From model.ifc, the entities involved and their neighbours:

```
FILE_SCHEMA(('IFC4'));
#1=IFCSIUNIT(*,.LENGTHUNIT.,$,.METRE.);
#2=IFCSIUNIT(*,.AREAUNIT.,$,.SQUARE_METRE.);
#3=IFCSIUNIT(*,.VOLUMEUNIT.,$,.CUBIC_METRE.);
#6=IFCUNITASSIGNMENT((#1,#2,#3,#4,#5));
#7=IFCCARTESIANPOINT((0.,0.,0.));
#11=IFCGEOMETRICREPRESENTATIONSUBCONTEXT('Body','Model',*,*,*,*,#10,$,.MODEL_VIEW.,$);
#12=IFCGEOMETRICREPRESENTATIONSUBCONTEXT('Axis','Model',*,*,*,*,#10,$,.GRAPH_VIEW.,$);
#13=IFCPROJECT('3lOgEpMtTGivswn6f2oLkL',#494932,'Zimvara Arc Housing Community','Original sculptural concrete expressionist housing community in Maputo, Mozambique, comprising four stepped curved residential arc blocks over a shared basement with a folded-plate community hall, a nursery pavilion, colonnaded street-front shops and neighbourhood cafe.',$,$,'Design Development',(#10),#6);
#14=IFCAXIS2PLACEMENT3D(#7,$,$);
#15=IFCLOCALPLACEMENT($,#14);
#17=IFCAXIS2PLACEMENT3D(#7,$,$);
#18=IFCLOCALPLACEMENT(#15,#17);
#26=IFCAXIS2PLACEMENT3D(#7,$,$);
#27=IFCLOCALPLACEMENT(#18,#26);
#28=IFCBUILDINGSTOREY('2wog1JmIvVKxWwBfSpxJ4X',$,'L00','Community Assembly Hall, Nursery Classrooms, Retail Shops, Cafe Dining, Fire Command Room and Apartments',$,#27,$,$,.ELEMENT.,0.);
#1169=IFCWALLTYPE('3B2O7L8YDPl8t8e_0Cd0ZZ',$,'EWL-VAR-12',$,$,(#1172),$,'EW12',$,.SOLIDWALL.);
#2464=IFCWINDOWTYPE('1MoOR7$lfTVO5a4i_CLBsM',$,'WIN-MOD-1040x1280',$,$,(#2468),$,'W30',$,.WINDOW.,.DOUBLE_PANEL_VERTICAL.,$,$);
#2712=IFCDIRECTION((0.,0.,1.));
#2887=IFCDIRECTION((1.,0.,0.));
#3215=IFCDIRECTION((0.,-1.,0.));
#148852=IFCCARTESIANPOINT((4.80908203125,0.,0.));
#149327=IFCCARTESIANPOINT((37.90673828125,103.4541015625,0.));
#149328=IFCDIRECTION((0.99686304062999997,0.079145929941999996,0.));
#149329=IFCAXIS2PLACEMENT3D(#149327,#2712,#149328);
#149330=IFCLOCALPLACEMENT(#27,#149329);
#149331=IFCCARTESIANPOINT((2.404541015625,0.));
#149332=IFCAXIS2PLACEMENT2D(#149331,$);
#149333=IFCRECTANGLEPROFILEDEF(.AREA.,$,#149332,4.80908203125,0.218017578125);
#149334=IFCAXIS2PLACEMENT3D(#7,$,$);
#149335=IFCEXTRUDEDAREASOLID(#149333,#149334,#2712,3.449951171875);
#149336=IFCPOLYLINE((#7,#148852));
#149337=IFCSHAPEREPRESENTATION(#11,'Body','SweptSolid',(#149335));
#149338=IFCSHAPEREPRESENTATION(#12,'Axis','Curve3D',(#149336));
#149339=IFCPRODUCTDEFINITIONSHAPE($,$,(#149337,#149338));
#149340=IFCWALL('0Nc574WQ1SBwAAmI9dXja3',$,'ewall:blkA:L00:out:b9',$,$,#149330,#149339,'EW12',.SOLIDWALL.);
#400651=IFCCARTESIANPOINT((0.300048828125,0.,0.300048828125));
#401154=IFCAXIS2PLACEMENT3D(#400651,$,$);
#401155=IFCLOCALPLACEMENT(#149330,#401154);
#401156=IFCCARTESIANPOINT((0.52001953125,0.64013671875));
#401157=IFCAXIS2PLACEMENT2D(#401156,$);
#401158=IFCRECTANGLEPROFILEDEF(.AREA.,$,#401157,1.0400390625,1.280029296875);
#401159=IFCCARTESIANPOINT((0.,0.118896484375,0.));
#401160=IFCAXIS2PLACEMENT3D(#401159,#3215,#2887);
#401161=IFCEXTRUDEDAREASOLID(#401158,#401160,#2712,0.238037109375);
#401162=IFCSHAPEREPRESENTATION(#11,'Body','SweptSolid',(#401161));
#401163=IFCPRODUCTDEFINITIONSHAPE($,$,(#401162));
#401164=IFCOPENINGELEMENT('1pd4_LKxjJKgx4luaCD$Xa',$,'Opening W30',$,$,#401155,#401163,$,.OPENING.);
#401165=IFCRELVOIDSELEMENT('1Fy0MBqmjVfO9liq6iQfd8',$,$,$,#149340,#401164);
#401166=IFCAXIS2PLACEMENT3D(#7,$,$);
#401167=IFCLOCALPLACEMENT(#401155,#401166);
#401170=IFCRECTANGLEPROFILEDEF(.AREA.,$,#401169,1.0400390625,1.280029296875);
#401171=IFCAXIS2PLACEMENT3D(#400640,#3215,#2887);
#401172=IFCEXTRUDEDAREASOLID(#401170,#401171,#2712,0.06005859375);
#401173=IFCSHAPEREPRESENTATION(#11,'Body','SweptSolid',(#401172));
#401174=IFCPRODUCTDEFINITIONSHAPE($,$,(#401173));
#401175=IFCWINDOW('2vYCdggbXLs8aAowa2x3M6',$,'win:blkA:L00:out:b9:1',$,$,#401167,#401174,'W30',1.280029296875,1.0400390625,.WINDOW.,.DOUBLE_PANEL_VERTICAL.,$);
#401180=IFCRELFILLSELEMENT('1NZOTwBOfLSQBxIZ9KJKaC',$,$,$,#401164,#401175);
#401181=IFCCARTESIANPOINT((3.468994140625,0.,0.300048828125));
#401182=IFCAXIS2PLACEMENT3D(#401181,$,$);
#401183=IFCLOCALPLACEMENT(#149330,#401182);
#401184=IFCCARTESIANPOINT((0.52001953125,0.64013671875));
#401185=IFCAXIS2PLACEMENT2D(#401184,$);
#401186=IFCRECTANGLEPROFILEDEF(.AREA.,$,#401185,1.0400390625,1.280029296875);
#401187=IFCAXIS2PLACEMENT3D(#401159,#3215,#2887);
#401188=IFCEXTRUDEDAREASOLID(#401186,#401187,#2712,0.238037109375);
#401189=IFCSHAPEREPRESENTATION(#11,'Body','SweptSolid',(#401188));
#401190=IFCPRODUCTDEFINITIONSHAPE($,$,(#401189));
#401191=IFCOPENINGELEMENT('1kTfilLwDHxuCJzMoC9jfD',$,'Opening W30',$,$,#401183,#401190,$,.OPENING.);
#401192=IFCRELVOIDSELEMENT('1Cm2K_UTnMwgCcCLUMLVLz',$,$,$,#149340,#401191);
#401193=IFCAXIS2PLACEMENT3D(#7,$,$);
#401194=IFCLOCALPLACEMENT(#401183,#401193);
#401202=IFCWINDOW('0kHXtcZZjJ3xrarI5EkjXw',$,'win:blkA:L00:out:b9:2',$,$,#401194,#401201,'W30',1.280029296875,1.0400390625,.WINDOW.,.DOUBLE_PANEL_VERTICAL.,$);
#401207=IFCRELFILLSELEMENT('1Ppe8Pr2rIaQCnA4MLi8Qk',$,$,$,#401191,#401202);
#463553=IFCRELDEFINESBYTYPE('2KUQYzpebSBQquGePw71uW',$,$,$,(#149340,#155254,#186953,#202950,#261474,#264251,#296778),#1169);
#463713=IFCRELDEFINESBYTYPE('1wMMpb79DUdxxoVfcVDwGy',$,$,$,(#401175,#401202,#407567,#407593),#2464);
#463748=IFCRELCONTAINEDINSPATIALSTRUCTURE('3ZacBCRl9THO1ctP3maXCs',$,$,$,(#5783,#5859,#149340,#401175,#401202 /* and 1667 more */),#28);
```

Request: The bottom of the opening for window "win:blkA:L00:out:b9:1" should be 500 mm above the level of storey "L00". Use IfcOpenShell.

```python
import numpy as np
import ifcopenshell
import ifcopenshell.api.geometry
import ifcopenshell.geom
import ifcopenshell.util.element
import ifcopenshell.util.placement
import ifcopenshell.util.shape
import ifcopenshell.util.unit

model = ifcopenshell.open("model.ifc")
unit_scale = ifcopenshell.util.unit.calculate_unit_scale(model)

window = model.by_guid("2vYCdggbXLs8aAowa2x3M6")
opening = window.FillsVoids[0].RelatingOpeningElement
storey = ifcopenshell.util.element.get_container(window, ifc_class="IfcBuildingStorey")
level = ifcopenshell.util.placement.get_local_placement(storey.ObjectPlacement)[2, 3]

# The opening's origin need not be at the sill, so measure its lowest point.
shape = ifcopenshell.geom.create_shape(ifcopenshell.geom.settings(), opening)
bottom = ifcopenshell.util.shape.get_shape_bottom_elevation(shape, shape.geometry) / unit_scale
dz = level + 0.5 - bottom

shift = np.array([0.0, 0.0, dz])
# The window is placed relative to its opening, so it follows when the opening moves.
matrix = ifcopenshell.util.placement.get_local_placement(opening.ObjectPlacement)
matrix[:3, 3] += shift
ifcopenshell.api.geometry.edit_object_placement(
    model, product=opening, matrix=matrix, is_si=False, should_transform_children=True
)

print(f"moved by {dz * unit_scale:+.3f} m")

model.write("model-out.ifc")
```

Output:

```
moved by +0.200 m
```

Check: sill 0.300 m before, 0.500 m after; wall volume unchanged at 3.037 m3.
